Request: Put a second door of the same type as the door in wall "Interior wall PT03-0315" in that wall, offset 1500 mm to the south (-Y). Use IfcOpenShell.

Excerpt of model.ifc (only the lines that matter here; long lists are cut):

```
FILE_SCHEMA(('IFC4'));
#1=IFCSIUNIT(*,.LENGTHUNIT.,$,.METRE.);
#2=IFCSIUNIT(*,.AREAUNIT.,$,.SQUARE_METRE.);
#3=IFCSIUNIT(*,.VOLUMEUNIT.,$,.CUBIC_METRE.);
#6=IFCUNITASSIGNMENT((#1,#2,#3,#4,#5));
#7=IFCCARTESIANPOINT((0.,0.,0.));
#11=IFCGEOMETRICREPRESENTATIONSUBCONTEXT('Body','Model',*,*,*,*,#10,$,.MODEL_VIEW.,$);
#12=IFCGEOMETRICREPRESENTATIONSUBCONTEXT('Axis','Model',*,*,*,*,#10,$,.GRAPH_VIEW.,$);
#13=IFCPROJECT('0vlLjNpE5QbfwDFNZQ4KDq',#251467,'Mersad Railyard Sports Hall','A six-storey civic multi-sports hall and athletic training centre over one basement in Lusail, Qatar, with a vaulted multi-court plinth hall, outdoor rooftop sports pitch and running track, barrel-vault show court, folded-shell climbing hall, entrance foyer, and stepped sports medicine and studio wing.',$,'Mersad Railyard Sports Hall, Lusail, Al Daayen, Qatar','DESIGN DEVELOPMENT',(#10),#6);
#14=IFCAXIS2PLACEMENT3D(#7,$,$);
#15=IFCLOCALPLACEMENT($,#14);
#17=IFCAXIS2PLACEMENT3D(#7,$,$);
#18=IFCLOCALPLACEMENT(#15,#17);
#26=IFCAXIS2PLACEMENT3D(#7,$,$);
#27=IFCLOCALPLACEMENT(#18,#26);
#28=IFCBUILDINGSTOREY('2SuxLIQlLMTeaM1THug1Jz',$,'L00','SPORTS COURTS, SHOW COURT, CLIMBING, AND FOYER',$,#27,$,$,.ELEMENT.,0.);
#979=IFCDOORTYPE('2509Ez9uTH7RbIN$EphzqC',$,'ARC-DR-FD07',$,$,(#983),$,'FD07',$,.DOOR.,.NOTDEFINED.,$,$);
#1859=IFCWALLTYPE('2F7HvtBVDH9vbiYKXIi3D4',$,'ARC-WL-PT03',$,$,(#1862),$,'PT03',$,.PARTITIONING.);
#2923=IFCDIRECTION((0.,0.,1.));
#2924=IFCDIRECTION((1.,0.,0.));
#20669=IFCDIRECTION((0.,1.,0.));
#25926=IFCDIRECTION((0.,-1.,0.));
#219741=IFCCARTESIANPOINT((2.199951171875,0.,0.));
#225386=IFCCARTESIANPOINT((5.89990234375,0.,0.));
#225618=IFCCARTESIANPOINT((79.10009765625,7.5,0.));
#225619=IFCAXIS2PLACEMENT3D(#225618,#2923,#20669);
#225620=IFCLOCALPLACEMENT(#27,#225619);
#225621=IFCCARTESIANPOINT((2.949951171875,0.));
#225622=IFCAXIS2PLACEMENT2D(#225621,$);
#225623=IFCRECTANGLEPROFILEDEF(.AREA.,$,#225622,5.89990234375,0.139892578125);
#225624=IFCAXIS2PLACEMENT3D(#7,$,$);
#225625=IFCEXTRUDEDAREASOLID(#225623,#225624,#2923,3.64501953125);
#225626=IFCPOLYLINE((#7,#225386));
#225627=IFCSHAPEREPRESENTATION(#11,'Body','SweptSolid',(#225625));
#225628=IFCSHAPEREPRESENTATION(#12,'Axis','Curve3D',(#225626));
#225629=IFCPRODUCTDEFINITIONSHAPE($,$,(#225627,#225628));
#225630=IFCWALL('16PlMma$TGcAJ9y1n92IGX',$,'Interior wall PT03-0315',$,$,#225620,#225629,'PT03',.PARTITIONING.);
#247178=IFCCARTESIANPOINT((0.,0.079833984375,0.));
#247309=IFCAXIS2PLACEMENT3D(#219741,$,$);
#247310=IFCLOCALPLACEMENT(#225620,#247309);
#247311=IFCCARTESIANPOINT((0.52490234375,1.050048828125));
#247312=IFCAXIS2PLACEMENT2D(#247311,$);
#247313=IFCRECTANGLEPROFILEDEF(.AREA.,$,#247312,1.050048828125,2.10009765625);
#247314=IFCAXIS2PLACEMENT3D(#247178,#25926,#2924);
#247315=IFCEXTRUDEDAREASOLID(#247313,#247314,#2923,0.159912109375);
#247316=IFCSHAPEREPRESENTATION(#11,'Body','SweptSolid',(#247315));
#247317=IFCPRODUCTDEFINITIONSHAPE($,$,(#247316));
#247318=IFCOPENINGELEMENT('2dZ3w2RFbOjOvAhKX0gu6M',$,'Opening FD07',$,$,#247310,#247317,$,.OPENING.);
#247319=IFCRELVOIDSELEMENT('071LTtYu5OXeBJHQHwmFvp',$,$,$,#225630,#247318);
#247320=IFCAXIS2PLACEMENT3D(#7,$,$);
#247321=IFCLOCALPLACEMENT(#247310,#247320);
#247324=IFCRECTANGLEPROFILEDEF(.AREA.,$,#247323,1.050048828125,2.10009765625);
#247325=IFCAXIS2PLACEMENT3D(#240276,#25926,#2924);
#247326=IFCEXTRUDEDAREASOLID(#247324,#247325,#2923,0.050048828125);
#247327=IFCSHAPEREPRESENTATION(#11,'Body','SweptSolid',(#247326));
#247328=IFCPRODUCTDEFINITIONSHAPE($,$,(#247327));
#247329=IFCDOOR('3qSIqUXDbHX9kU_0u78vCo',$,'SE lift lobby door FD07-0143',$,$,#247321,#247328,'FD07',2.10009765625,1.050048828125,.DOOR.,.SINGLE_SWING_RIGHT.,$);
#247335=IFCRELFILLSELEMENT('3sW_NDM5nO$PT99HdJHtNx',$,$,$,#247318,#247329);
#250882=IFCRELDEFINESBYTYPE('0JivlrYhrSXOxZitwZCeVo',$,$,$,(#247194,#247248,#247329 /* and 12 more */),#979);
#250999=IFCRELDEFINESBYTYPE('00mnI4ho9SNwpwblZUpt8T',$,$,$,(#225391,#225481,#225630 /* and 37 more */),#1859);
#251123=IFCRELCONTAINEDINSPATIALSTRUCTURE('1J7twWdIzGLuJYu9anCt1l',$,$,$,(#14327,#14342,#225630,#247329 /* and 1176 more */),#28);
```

```python
import ifcopenshell
import ifcopenshell.api.feature
import ifcopenshell.api.geometry
import ifcopenshell.api.root
import ifcopenshell.geom
import ifcopenshell.util.element
import ifcopenshell.util.placement
import ifcopenshell.util.shape

model = ifcopenshell.open("model.ifc")
settings = ifcopenshell.geom.settings()


def volume(element):
    """Net volume in cubic metres, openings subtracted."""
    shape = ifcopenshell.geom.create_shape(settings, element)
    return ifcopenshell.util.shape.get_volume(shape.geometry)


door = model.by_guid("3qSIqUXDbHX9kU_0u78vCo")
opening = door.FillsVoids[0].RelatingOpeningElement
wall = opening.VoidsElements[0].RelatingBuildingElement
before = volume(wall)
shift = ifcopenshell.util.placement.get_local_placement(wall.ObjectPlacement)[:3, 0] * -1.5

# copy_class copies the void relationship, type, container and properties, but no geometry.
new_opening = ifcopenshell.api.root.copy_class(model, product=opening)
new_opening.Representation = ifcopenshell.util.element.copy_deep(
    model, opening.Representation, exclude=["IfcGeometricRepresentationContext", "IfcRepresentationMap"]
)
new_door = ifcopenshell.api.root.copy_class(model, product=door)
new_door.Representation = ifcopenshell.util.element.copy_deep(
    model, door.Representation, exclude=["IfcGeometricRepresentationContext", "IfcRepresentationMap"]
)
new_door.Tag = None
ifcopenshell.api.feature.add_filling(model, opening=new_opening, element=new_door)

for old, new in ((opening, new_opening), (door, new_door)):
    matrix = ifcopenshell.util.placement.get_local_placement(old.ObjectPlacement)
    matrix[:3, 3] += shift
    ifcopenshell.api.geometry.edit_object_placement(model, product=new, matrix=matrix, is_si=False)

after = volume(wall)

print(f"wall volume {before:.3f} -> {after:.3f} m3")

model.write("model_edited.ifc")
```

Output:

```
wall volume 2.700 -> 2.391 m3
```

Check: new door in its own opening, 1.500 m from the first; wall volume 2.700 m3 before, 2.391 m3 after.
